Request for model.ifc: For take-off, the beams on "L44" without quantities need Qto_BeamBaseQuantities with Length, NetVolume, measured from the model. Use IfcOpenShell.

First a look at what the model holds.

```python
import ifcopenshell
import ifcopenshell.util.element
import ifcopenshell.util.unit

model = ifcopenshell.open("model.ifc")
print(model.schema)
for unit_type in ("LENGTHUNIT", "AREAUNIT", "VOLUMEUNIT"):
    print(unit_type, ifcopenshell.util.unit.calculate_unit_scale(model, unit_type))
storey = next(s for s in model.by_type("IfcBuildingStorey") if s.Name == "L44")
beams = [e for e in ifcopenshell.util.element.get_decomposition(storey) if e.is_a("IfcBeam")]
for e in sorted(beams, key=lambda e: e.id()):
    print(e.id(), e.is_a(), e.Name, list(ifcopenshell.util.element.get_psets(e, qtos_only=True)), sep=" | ")
```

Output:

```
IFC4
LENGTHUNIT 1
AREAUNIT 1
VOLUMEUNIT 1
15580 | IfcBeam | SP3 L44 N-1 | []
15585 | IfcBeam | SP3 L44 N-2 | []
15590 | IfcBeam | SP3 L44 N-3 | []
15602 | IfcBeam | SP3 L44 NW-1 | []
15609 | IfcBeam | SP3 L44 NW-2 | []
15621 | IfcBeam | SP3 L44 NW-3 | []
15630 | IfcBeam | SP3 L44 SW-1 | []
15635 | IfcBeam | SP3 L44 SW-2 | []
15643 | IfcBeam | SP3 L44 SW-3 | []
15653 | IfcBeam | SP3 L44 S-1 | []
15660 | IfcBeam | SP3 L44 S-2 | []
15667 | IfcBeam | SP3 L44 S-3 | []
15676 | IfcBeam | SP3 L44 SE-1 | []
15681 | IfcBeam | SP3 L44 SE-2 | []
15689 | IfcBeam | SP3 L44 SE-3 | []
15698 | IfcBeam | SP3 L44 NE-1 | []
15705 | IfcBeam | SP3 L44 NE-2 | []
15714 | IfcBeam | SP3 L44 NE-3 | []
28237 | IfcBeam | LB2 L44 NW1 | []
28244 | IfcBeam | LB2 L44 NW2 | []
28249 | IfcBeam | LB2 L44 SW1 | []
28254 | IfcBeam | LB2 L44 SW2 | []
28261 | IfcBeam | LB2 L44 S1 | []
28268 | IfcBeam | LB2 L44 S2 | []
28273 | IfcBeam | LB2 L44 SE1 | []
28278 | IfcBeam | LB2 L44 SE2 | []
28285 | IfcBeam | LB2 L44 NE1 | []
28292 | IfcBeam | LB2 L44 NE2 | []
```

```python
import ifcopenshell
import ifcopenshell.api.pset
import ifcopenshell.geom
import ifcopenshell.util.element
import ifcopenshell.util.shape
import ifcopenshell.util.unit

model = ifcopenshell.open("model.ifc")
unit_scale = ifcopenshell.util.unit.calculate_unit_scale(model)
volume_scale = ifcopenshell.util.unit.calculate_unit_scale(model, "VOLUMEUNIT")
settings = ifcopenshell.geom.settings()

storey = next(s for s in model.by_type("IfcBuildingStorey") if s.Name == "L44")
beams = [e for e in ifcopenshell.util.element.get_decomposition(storey) if e.is_a("IfcBeam")]

for e in sorted(beams, key=lambda e: e.id()):
    if ifcopenshell.util.element.get_psets(e, qtos_only=True, should_inherit=False):
        continue
    # Geometry comes back in metres, in the element's own axes.
    shape = ifcopenshell.geom.create_shape(settings, e)
    values = {
        "Length": ifcopenshell.util.shape.get_max_xyz(shape.geometry) / unit_scale,
        "NetVolume": ifcopenshell.util.shape.get_volume(shape.geometry) / volume_scale,
    }
    qto = ifcopenshell.api.pset.add_qto(model, product=e, name="Qto_BeamBaseQuantities")
    ifcopenshell.api.pset.edit_qto(model, qto=qto, properties=values)
    print(e.id(), {k: round(v, 3) for k, v in values.items()})

model.write("model_updated.ifc")
```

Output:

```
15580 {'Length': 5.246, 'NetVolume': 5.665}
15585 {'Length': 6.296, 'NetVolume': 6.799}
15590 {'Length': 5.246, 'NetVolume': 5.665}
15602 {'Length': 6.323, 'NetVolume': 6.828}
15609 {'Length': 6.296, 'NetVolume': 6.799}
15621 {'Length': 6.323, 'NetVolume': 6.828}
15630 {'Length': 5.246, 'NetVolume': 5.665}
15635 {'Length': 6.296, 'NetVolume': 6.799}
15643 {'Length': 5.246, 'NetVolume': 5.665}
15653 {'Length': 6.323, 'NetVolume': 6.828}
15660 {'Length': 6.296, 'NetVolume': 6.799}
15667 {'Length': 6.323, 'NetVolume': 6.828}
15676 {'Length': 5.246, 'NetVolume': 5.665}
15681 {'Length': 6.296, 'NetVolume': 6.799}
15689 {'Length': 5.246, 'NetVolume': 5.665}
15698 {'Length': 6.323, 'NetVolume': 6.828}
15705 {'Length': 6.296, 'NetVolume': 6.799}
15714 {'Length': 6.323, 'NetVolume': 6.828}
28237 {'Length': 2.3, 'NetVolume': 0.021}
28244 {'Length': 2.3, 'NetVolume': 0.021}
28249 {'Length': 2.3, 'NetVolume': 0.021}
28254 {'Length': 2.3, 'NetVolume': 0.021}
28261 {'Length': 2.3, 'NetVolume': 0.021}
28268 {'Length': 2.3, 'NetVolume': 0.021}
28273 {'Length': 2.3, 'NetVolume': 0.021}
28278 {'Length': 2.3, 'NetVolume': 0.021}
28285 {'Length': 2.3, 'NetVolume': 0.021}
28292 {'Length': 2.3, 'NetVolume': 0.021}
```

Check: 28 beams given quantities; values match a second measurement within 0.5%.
